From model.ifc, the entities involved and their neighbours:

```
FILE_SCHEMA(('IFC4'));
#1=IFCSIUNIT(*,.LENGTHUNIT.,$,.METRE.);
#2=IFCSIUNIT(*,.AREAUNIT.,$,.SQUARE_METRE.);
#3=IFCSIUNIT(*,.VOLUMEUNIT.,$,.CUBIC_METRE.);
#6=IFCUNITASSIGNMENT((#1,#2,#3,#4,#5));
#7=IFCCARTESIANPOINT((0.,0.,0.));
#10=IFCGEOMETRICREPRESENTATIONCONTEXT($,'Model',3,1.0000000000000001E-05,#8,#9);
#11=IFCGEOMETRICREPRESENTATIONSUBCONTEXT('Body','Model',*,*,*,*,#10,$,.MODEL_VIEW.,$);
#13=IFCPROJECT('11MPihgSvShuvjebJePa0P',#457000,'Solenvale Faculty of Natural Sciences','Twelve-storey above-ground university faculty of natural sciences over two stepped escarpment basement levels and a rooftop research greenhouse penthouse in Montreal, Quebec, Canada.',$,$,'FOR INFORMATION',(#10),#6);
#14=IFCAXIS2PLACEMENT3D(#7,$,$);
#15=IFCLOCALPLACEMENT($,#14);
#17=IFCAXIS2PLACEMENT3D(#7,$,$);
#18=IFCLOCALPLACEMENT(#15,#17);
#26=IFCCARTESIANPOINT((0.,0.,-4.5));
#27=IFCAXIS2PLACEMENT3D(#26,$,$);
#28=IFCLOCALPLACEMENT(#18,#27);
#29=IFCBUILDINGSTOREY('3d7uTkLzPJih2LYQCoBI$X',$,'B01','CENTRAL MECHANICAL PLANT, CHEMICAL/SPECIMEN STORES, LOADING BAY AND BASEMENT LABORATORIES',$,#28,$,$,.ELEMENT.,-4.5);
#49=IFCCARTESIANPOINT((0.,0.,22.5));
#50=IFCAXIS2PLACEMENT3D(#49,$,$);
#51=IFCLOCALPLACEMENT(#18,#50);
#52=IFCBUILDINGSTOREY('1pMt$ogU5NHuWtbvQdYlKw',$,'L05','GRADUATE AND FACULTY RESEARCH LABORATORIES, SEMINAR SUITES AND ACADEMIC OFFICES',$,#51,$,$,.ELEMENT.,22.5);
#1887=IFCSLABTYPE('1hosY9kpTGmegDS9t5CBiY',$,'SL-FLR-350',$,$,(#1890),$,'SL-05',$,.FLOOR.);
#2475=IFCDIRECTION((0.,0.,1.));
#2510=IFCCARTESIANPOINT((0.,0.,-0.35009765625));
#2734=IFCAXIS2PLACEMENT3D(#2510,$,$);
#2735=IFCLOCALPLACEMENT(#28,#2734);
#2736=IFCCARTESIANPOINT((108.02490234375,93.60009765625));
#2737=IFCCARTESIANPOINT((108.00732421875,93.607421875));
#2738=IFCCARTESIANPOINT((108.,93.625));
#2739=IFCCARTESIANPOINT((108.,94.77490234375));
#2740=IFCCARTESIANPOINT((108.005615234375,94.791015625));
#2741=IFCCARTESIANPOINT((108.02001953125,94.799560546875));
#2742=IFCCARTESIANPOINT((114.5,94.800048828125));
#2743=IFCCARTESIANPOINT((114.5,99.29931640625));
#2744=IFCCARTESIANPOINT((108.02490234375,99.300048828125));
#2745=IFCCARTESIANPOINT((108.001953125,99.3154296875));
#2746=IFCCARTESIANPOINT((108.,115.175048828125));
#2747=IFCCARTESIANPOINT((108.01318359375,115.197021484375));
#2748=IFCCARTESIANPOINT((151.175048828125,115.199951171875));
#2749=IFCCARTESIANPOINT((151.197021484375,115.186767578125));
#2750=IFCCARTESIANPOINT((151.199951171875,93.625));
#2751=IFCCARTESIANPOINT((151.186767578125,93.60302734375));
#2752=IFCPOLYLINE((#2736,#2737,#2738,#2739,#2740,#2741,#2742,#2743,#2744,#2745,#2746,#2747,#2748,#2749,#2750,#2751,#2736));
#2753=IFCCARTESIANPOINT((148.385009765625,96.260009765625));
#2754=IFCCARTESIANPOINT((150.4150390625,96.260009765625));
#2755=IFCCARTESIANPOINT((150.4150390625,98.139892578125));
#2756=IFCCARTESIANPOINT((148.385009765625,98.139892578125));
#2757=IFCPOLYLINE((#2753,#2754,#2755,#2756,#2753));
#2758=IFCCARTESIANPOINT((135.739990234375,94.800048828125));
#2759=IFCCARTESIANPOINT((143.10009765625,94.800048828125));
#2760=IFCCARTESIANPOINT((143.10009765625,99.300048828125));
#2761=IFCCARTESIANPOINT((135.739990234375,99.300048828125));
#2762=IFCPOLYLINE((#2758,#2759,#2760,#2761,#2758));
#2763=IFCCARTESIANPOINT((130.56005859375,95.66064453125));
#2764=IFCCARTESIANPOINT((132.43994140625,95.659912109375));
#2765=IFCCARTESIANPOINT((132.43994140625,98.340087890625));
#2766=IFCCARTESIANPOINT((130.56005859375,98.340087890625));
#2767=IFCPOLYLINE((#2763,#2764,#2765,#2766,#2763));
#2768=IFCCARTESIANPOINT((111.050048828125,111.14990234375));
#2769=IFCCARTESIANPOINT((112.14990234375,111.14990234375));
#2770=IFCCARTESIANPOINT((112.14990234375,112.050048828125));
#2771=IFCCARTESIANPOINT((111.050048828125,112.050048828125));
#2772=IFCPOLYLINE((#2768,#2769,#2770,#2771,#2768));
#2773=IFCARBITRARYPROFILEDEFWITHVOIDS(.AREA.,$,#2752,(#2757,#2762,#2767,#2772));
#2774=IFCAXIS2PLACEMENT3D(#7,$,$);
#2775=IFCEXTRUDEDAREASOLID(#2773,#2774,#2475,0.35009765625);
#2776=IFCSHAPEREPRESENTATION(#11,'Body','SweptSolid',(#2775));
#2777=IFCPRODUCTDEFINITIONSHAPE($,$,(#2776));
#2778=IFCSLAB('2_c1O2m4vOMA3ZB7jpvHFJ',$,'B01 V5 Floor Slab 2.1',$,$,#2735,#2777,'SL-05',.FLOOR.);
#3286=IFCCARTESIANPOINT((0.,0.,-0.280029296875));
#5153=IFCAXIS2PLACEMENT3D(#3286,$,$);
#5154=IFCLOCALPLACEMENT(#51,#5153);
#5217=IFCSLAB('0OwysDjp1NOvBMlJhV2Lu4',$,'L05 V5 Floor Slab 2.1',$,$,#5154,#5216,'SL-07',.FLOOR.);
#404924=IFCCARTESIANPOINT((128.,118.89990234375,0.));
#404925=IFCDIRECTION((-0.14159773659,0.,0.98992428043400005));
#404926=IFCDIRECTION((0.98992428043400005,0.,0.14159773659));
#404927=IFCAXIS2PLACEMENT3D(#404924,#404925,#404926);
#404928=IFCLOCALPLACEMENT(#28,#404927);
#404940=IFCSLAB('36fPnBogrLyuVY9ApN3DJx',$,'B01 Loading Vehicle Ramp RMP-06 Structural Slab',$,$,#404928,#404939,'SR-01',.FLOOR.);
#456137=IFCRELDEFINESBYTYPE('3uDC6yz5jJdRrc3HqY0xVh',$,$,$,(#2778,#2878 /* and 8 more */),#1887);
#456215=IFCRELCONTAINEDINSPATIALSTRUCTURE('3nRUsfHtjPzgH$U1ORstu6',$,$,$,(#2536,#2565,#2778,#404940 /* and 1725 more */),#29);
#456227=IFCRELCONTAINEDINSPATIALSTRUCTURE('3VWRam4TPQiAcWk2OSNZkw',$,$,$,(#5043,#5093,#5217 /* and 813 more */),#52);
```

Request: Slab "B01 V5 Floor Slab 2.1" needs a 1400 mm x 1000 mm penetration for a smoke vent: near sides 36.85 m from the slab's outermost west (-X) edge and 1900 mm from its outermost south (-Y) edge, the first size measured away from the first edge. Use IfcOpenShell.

```python
import numpy as np
import ifcopenshell
import ifcopenshell.api.feature
import ifcopenshell.api.geometry
import ifcopenshell.api.root
import ifcopenshell.geom
import ifcopenshell.util.placement
import ifcopenshell.util.representation
import ifcopenshell.util.shape
import ifcopenshell.util.unit

model = ifcopenshell.open("model.ifc")
unit_scale = ifcopenshell.util.unit.calculate_unit_scale(model)
settings = ifcopenshell.geom.settings()


def volume(element):
    """Net volume in cubic metres, openings subtracted."""
    shape = ifcopenshell.geom.create_shape(settings, element)
    return ifcopenshell.util.shape.get_volume(shape.geometry)


slab = model.by_guid("2_c1O2m4vOMA3ZB7jpvHFJ")
before = volume(slab)

# Extent in the slab's own axes, in metres. The edges named are its -X and -Y sides.
slab_shape = ifcopenshell.geom.create_shape(settings, slab)
vertices = ifcopenshell.util.shape.get_vertices(slab_shape.geometry)
x_min, y_min, bottom = vertices.min(axis=0)
top = vertices[:, 2].max()

opening = ifcopenshell.api.root.create_entity(model, ifc_class="IfcOpeningElement", name="Smoke vent opening", predefined_type="OPENING")
context = ifcopenshell.util.representation.get_context(model, "Model", "Body", "MODEL_VIEW")
width, depth = 1.4, 1
outline = [(0.0, 0.0), (width, 0.0), (width, depth), (0.0, depth), (0.0, 0.0)]
# Overshoot both faces by 50 mm so the cut is clean.
shape = ifcopenshell.api.geometry.add_slab_representation(
    model, context=context, depth=top - bottom + 0.1, polyline=outline
)
ifcopenshell.api.geometry.assign_representation(model, product=opening, representation=shape)

matrix = ifcopenshell.util.placement.get_local_placement(slab.ObjectPlacement)
matrix[:, 3] = matrix @ np.append(np.array([x_min + 36.85, y_min + 1.9, bottom - 0.05]) / unit_scale, 1.0)
ifcopenshell.api.geometry.edit_object_placement(model, product=opening, matrix=matrix, is_si=False)
ifcopenshell.api.feature.add_feature(model, feature=opening, element=slab)

after = volume(slab)

print(f"slab volume {before:.3f} -> {after:.3f} m3")

model.write("model_edited.ifc")
```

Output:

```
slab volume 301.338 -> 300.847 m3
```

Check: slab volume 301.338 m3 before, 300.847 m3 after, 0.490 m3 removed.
